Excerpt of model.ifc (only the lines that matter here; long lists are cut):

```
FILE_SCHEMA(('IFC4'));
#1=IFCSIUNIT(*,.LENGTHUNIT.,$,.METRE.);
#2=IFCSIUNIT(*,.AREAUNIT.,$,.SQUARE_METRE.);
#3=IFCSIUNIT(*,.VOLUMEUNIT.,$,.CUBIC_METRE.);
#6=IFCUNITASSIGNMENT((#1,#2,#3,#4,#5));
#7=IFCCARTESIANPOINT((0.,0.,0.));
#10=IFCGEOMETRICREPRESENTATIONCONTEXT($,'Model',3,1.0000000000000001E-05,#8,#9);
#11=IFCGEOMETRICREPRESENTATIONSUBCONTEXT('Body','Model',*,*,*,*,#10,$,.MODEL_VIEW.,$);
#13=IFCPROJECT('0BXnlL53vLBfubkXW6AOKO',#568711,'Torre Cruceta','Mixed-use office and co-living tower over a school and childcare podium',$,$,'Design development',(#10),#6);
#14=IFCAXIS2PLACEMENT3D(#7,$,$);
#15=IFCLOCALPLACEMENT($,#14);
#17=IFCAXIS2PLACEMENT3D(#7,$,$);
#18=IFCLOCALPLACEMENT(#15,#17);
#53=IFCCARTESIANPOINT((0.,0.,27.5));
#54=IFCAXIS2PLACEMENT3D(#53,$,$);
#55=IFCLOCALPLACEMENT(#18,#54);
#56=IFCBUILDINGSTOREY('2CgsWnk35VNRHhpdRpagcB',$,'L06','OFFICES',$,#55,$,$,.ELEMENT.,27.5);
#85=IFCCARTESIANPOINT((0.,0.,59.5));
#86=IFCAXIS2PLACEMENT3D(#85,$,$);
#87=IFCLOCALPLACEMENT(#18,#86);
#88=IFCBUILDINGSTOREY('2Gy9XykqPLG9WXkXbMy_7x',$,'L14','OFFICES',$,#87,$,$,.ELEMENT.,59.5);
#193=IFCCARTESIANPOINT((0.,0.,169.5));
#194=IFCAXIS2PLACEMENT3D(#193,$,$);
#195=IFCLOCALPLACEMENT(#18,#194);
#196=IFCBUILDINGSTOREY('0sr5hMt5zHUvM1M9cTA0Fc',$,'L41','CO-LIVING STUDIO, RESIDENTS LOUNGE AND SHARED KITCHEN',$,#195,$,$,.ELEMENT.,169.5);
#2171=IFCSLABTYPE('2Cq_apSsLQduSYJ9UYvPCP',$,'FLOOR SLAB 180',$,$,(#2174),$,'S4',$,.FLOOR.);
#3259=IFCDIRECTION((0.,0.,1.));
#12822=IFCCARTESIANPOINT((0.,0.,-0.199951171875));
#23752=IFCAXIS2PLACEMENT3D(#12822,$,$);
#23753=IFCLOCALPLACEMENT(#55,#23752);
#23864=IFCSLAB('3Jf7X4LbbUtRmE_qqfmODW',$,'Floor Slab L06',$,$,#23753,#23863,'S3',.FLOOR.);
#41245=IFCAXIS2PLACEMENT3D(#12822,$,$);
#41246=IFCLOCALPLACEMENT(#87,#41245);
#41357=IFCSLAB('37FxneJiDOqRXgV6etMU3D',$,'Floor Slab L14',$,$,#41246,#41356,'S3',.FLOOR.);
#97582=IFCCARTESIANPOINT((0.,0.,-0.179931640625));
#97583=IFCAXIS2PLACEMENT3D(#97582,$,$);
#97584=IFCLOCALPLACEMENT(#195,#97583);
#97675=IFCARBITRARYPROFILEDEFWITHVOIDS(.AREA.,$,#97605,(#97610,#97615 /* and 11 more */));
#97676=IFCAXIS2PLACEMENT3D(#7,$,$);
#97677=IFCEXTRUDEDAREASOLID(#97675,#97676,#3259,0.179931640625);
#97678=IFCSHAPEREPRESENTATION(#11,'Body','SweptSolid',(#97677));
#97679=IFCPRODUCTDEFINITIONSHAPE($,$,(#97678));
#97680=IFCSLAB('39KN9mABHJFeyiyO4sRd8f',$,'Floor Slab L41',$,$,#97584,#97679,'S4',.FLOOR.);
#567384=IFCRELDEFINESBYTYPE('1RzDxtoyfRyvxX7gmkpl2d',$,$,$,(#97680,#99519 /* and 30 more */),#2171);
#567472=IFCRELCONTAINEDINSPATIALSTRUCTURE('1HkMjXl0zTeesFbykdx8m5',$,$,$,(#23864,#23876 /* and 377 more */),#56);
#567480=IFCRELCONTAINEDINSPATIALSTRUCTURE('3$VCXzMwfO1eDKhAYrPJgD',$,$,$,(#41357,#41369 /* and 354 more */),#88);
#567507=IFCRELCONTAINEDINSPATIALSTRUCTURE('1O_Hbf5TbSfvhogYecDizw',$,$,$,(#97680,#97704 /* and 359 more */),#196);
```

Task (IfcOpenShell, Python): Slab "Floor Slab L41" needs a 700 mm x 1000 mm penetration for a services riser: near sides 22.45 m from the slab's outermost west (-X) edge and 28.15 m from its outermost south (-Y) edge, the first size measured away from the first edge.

```python
import numpy as np
import ifcopenshell
import ifcopenshell.api.feature
import ifcopenshell.api.geometry
import ifcopenshell.api.root
import ifcopenshell.geom
import ifcopenshell.util.placement
import ifcopenshell.util.representation
import ifcopenshell.util.shape
import ifcopenshell.util.unit

model = ifcopenshell.open("model.ifc")
unit_scale = ifcopenshell.util.unit.calculate_unit_scale(model)
settings = ifcopenshell.geom.settings()


def volume(element):
    """Net volume in cubic metres, openings subtracted."""
    shape = ifcopenshell.geom.create_shape(settings, element)
    return ifcopenshell.util.shape.get_volume(shape.geometry)


slab = model.by_guid("39KN9mABHJFeyiyO4sRd8f")
before = volume(slab)

# Extent in the slab's own axes, in metres. The edges named are its -X and -Y sides.
slab_shape = ifcopenshell.geom.create_shape(settings, slab)
vertices = ifcopenshell.util.shape.get_vertices(slab_shape.geometry)
x_min, y_min, bottom = vertices.min(axis=0)
top = vertices[:, 2].max()

opening = ifcopenshell.api.root.create_entity(model, ifc_class="IfcOpeningElement", name="Services riser opening", predefined_type="OPENING")
context = ifcopenshell.util.representation.get_context(model, "Model", "Body", "MODEL_VIEW")
width, depth = 0.7, 1
outline = [(0.0, 0.0), (width, 0.0), (width, depth), (0.0, depth), (0.0, 0.0)]
# Overshoot both faces by 50 mm so the cut is clean.
shape = ifcopenshell.api.geometry.add_slab_representation(
    model, context=context, depth=top - bottom + 0.1, polyline=outline
)
ifcopenshell.api.geometry.assign_representation(model, product=opening, representation=shape)

matrix = ifcopenshell.util.placement.get_local_placement(slab.ObjectPlacement)
matrix[:, 3] = matrix @ np.append(np.array([x_min + 22.45, y_min + 28.15, bottom - 0.05]) / unit_scale, 1.0)
ifcopenshell.api.geometry.edit_object_placement(model, product=opening, matrix=matrix, is_si=False)
ifcopenshell.api.feature.add_feature(model, feature=opening, element=slab)

after = volume(slab)

print(f"slab volume {before:.3f} -> {after:.3f} m3")

model.write("model_rev.ifc")
```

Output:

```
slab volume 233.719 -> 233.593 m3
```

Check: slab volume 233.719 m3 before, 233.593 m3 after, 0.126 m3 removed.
